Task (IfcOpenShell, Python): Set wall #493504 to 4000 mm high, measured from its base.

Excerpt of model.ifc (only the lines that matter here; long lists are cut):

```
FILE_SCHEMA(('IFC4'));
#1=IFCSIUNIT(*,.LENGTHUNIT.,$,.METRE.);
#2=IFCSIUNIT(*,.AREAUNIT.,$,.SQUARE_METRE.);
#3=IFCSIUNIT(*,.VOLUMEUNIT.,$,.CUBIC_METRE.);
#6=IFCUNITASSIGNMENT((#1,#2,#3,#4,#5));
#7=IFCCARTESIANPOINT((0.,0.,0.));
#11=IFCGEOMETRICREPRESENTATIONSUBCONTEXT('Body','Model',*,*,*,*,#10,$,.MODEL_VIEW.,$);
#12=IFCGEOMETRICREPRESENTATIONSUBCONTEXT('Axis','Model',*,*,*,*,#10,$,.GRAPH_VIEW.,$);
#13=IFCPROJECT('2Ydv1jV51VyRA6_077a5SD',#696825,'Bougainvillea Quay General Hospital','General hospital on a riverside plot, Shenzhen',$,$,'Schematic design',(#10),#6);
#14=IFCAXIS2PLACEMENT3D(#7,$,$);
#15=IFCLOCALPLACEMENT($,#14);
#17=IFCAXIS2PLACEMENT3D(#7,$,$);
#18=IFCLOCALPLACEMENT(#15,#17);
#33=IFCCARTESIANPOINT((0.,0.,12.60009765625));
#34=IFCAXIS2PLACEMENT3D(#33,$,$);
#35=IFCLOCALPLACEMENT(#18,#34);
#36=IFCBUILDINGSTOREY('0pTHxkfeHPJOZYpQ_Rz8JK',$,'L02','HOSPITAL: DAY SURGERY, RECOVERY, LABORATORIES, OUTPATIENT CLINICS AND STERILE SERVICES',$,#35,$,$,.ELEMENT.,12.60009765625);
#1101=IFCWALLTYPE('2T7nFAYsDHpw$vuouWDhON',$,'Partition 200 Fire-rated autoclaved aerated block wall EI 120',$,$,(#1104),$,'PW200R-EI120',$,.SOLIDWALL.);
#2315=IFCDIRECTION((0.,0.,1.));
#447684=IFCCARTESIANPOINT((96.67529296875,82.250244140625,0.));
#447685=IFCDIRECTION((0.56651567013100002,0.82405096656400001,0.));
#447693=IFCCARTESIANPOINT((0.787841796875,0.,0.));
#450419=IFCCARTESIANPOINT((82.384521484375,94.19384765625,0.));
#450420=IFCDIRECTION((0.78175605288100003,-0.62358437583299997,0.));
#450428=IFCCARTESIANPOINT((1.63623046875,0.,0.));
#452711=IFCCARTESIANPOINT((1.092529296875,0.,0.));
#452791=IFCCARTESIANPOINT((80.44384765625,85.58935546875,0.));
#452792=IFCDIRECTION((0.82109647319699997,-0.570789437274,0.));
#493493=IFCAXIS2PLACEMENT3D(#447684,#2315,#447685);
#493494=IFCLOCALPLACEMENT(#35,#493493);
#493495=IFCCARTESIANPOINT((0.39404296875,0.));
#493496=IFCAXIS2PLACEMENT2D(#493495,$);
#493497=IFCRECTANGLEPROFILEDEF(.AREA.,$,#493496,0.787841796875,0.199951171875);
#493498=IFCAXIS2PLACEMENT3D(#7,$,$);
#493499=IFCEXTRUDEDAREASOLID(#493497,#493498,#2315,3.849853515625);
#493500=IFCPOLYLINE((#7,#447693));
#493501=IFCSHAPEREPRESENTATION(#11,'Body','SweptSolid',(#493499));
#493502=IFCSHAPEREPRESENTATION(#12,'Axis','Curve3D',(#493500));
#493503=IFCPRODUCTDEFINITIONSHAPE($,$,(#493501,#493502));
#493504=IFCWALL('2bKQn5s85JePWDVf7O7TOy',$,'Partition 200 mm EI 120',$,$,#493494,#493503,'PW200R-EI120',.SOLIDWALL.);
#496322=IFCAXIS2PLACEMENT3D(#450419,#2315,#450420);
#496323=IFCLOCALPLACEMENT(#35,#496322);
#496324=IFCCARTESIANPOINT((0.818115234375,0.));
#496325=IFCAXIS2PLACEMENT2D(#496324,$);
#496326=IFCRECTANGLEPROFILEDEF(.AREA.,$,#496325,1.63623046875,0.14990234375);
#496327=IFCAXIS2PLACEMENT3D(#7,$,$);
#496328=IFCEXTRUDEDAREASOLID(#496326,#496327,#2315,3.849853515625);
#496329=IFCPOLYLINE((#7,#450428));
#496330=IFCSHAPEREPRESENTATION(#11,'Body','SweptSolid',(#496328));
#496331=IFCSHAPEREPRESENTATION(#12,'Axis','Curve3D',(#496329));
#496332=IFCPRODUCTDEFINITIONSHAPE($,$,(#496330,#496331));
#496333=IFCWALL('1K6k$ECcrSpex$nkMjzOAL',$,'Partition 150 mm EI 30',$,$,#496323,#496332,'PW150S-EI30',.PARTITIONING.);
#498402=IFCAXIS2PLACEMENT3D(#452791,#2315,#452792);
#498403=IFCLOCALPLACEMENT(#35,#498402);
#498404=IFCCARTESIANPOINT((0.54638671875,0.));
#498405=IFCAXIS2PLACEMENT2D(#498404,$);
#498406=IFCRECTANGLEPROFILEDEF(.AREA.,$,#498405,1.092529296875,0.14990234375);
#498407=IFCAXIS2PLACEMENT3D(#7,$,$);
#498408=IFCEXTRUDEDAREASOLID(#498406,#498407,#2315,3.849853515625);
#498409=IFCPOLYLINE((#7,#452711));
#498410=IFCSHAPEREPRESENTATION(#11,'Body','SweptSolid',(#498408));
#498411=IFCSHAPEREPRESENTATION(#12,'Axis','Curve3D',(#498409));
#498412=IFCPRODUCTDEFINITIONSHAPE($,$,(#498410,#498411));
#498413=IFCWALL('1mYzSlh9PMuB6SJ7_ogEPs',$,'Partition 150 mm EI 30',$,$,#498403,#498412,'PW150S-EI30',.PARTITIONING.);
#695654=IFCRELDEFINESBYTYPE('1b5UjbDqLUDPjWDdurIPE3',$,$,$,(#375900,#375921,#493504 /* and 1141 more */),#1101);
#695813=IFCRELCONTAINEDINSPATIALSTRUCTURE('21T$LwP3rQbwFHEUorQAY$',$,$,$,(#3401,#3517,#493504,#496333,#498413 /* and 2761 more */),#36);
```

```python
import ifcopenshell
import ifcopenshell.geom
import ifcopenshell.util.representation
import ifcopenshell.util.shape

model = ifcopenshell.open("model.ifc")
settings = ifcopenshell.geom.settings()


def volume(element):
    """Net volume in cubic metres, openings subtracted."""
    shape = ifcopenshell.geom.create_shape(settings, element)
    return ifcopenshell.util.shape.get_volume(shape.geometry)


wall = model.by_guid("2bKQn5s85JePWDVf7O7TOy")
before = volume(wall)

body = ifcopenshell.util.representation.get_representation(wall, "Model", "Body")
solid = body.Items[0]
old_height = solid.Depth
solid.Depth = 4.0
after = volume(wall)

print(f"height {old_height:g} -> {solid.Depth:g}, volume {before:.3f} -> {after:.3f} m3")

model.write("model_edited.ifc")
```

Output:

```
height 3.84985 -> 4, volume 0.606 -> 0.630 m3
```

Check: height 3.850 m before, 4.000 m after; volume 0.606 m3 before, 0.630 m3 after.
